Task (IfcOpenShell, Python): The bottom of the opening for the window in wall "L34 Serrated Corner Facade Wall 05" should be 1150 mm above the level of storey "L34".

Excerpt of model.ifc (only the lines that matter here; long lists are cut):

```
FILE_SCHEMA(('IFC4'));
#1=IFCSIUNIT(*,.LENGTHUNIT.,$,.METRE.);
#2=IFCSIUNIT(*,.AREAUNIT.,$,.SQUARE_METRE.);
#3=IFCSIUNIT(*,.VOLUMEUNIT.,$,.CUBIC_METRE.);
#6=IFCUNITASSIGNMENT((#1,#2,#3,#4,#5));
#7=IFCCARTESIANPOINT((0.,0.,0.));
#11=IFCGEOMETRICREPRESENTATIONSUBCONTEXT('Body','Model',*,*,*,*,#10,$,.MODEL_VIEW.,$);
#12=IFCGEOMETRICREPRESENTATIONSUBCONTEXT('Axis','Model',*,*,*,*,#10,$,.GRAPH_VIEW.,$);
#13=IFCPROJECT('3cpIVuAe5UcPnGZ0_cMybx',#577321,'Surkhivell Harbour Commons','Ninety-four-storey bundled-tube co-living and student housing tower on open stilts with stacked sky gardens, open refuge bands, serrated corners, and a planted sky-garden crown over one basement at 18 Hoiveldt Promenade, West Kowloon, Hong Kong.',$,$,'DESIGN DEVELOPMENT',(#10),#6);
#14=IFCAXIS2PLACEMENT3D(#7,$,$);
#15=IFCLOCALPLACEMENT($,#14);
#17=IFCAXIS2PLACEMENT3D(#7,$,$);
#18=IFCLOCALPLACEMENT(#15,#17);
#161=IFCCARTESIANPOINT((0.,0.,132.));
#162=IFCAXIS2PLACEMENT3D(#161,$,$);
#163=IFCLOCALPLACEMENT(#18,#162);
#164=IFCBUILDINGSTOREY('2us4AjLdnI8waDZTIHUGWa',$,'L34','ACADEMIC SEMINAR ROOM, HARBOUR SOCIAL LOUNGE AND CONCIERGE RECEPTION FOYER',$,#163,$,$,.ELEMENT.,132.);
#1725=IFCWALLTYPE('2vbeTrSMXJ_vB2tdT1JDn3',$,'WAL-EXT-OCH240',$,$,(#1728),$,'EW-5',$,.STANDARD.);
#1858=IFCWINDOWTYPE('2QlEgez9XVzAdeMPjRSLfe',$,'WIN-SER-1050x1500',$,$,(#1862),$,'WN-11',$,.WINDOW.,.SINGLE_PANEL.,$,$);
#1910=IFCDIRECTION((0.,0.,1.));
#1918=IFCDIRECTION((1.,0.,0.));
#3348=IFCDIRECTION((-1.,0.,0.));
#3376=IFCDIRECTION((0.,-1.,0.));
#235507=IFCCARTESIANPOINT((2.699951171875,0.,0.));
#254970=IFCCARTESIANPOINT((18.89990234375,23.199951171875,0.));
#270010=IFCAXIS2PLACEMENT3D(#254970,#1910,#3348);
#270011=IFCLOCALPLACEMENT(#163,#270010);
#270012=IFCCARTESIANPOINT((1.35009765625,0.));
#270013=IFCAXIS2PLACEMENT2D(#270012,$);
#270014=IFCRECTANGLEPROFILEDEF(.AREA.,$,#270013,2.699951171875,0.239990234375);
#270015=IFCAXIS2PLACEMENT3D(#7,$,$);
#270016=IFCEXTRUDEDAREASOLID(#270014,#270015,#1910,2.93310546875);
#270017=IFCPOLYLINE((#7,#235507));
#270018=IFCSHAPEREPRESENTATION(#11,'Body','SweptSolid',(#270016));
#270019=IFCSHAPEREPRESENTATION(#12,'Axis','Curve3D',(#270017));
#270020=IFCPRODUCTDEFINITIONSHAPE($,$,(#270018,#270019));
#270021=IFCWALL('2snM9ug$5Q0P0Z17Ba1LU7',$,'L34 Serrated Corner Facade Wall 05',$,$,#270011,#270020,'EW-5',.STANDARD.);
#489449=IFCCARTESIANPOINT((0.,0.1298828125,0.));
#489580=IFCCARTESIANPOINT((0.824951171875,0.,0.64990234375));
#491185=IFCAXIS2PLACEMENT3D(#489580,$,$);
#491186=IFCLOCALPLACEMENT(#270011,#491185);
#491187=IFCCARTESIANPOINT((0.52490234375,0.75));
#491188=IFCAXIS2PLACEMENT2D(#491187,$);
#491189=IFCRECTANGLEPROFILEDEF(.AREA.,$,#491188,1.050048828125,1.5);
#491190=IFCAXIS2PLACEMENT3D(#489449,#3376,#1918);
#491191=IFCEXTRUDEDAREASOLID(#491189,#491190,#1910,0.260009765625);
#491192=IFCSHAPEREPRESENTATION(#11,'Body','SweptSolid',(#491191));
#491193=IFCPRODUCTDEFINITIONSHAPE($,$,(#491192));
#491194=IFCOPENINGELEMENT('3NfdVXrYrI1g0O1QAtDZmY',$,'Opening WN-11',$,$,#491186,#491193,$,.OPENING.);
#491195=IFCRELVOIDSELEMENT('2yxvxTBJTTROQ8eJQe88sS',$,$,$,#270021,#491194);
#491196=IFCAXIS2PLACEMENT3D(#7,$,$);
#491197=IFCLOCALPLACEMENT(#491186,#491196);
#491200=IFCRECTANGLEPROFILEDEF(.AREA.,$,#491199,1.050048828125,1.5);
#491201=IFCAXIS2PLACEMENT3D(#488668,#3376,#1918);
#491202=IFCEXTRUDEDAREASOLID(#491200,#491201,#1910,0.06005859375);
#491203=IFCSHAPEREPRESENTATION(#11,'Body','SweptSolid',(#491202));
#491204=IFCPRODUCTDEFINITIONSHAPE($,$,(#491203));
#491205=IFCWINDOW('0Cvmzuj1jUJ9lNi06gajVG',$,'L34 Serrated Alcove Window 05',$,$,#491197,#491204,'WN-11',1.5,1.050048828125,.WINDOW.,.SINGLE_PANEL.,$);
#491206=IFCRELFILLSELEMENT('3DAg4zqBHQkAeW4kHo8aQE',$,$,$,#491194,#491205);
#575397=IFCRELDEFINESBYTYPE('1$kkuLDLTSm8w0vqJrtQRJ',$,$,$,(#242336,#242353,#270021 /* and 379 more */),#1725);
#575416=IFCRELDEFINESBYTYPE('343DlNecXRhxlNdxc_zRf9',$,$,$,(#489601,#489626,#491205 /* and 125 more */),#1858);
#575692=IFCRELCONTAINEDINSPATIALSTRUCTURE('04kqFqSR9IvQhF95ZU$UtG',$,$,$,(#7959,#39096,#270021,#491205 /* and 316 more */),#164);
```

```python
import numpy as np
import ifcopenshell
import ifcopenshell.api.geometry
import ifcopenshell.geom
import ifcopenshell.util.element
import ifcopenshell.util.placement
import ifcopenshell.util.shape
import ifcopenshell.util.unit

model = ifcopenshell.open("model.ifc")
unit_scale = ifcopenshell.util.unit.calculate_unit_scale(model)

window = model.by_id(491205)
opening = window.FillsVoids[0].RelatingOpeningElement
storey = ifcopenshell.util.element.get_container(window, ifc_class="IfcBuildingStorey")
level = ifcopenshell.util.placement.get_local_placement(storey.ObjectPlacement)[2, 3]

# The opening's origin need not be at the sill, so measure its lowest point.
shape = ifcopenshell.geom.create_shape(ifcopenshell.geom.settings(), opening)
bottom = ifcopenshell.util.shape.get_shape_bottom_elevation(shape, shape.geometry) / unit_scale
dz = level + 1.15 / unit_scale - bottom

shift = np.array([0.0, 0.0, dz])
# The window is placed relative to its opening, so it follows when the opening moves.
matrix = ifcopenshell.util.placement.get_local_placement(opening.ObjectPlacement)
matrix[:3, 3] += shift
ifcopenshell.api.geometry.edit_object_placement(
    model, product=opening, matrix=matrix, is_si=False, should_transform_children=True
)

print(f"moved by {dz * unit_scale:+.3f} m")

model.write("model_edited.ifc")
```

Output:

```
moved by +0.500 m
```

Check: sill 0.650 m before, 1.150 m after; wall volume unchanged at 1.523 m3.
